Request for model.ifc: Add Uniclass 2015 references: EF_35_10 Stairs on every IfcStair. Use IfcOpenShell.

First a look at what the model holds.

```python
import ifcopenshell

model = ifcopenshell.open("model.ifc")
print(model.schema)
print("classifications:", [c.Name for c in model.by_type("IfcClassification")])
for ifc_class in ("IfcDoor", "IfcRoof", "IfcStair", "IfcWall", "IfcWindow"):
    print(ifc_class, len(model.by_type(ifc_class)))
```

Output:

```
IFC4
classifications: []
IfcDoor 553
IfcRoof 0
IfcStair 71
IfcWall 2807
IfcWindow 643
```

```python
import ifcopenshell
import ifcopenshell.api.classification

model = ifcopenshell.open("model.ifc")

system = ifcopenshell.api.classification.add_classification(model, classification="Uniclass 2015")

codes = {
    "IfcStair": ("EF_35_10", "Stairs"),
}
for ifc_class, (code, name) in codes.items():
    products = model.by_type(ifc_class)
    ifcopenshell.api.classification.add_reference(
        model, products=products, classification=system, identification=code, name=name
    )
    print(code, len(products))

model.write("model_edited.ifc")
```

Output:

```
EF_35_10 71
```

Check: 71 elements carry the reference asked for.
